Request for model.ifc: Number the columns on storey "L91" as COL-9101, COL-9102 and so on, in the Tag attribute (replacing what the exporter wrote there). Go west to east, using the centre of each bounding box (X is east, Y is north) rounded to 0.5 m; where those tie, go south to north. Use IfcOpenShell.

First a look at what the model holds.

```python
import ifcopenshell
import ifcopenshell.util.element
import ifcopenshell.util.placement

model = ifcopenshell.open("model.ifc")
print(model.schema)
storey = next(s for s in model.by_type("IfcBuildingStorey") if s.Name == "L91")
columns = [e for e in ifcopenshell.util.element.get_decomposition(storey) if e.is_a("IfcColumn")]
for e in sorted(columns, key=lambda e: e.id()):
    origin = ifcopenshell.util.placement.get_local_placement(e.ObjectPlacement)[:3, 3]
    print(e.id(), e.Tag, e.Name, origin.round(2) + 0.0, sep=" | ")
```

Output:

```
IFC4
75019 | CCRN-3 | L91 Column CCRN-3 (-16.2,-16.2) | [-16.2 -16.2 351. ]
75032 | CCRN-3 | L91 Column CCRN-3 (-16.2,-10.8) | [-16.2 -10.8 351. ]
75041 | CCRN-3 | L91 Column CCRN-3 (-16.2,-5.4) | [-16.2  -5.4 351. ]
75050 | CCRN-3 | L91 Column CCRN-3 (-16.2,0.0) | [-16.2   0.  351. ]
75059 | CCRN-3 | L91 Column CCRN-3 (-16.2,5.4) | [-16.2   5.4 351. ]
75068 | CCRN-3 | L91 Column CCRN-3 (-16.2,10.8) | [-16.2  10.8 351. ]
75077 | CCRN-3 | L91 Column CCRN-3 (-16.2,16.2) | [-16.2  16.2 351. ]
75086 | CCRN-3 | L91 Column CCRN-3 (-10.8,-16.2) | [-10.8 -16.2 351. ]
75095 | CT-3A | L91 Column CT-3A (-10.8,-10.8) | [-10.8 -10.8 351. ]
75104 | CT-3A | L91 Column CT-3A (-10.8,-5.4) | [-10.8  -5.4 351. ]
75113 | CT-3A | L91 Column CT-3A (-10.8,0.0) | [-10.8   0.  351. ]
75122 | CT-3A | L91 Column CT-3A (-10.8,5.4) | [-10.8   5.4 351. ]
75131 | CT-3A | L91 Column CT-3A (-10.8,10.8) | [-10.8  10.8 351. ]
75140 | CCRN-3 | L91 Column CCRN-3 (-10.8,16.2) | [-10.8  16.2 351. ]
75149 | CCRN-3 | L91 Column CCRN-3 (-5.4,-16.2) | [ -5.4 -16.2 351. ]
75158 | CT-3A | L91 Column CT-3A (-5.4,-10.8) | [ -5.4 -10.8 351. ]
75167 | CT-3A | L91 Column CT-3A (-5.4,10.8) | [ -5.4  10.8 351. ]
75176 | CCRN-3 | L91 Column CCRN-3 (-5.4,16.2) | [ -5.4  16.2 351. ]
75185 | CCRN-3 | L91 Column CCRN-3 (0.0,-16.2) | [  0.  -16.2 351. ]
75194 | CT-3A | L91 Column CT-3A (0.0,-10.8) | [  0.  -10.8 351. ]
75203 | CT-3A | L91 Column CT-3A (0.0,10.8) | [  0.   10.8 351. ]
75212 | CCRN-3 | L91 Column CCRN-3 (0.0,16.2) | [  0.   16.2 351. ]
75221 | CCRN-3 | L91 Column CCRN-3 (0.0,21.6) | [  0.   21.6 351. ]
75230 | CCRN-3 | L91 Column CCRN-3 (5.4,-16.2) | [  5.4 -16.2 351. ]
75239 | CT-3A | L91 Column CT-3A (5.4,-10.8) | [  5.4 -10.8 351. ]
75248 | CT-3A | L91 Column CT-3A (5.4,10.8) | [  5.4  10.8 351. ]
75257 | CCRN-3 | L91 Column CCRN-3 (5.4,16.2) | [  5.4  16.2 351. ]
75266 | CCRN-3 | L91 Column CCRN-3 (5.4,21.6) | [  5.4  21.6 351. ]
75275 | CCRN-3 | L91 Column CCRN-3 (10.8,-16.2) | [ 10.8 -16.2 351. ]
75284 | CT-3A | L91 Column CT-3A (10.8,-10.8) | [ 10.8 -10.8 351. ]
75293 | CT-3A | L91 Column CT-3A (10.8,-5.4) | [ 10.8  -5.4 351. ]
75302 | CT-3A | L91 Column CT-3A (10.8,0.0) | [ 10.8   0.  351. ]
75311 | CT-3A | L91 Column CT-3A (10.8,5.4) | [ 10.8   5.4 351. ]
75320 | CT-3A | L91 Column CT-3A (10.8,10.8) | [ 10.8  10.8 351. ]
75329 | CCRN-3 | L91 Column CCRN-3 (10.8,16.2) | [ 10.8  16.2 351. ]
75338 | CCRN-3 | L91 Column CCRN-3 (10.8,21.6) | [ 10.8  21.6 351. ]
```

```python
import ifcopenshell
import ifcopenshell.geom
import ifcopenshell.util.element
import ifcopenshell.util.shape

model = ifcopenshell.open("model.ifc")
settings = ifcopenshell.geom.settings()
settings.set("use-world-coords", True)


def centre(element):
    shape = ifcopenshell.geom.create_shape(settings, element)
    return ifcopenshell.util.shape.get_bbox_centroid(shape.geometry)


storey = next(s for s in model.by_type("IfcBuildingStorey") if s.Name == "L91")
columns = [e for e in ifcopenshell.util.element.get_decomposition(storey) if e.is_a("IfcColumn")]

# Insertion points can sit at a corner or the storey origin, so sort by the geometry (in metres).
centres = {e: centre(e) for e in columns}
columns.sort(key=lambda e: (round(centres[e][0] / 0.5), centres[e][1]))

for i, e in enumerate(columns, start=1):
    number = f"COL-91{i:02d}"
    e.Tag = number
    print(e.id(), number)

model.write("model_v2.ifc")
```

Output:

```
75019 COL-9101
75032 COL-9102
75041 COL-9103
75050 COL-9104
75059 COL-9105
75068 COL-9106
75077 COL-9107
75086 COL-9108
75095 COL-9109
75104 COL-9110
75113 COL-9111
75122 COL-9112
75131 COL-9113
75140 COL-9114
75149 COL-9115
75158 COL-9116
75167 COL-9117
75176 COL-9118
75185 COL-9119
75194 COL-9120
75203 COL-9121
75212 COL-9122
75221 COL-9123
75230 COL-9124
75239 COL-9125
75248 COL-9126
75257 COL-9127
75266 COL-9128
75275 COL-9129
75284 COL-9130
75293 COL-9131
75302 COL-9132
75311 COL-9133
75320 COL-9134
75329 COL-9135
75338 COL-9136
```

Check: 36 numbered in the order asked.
